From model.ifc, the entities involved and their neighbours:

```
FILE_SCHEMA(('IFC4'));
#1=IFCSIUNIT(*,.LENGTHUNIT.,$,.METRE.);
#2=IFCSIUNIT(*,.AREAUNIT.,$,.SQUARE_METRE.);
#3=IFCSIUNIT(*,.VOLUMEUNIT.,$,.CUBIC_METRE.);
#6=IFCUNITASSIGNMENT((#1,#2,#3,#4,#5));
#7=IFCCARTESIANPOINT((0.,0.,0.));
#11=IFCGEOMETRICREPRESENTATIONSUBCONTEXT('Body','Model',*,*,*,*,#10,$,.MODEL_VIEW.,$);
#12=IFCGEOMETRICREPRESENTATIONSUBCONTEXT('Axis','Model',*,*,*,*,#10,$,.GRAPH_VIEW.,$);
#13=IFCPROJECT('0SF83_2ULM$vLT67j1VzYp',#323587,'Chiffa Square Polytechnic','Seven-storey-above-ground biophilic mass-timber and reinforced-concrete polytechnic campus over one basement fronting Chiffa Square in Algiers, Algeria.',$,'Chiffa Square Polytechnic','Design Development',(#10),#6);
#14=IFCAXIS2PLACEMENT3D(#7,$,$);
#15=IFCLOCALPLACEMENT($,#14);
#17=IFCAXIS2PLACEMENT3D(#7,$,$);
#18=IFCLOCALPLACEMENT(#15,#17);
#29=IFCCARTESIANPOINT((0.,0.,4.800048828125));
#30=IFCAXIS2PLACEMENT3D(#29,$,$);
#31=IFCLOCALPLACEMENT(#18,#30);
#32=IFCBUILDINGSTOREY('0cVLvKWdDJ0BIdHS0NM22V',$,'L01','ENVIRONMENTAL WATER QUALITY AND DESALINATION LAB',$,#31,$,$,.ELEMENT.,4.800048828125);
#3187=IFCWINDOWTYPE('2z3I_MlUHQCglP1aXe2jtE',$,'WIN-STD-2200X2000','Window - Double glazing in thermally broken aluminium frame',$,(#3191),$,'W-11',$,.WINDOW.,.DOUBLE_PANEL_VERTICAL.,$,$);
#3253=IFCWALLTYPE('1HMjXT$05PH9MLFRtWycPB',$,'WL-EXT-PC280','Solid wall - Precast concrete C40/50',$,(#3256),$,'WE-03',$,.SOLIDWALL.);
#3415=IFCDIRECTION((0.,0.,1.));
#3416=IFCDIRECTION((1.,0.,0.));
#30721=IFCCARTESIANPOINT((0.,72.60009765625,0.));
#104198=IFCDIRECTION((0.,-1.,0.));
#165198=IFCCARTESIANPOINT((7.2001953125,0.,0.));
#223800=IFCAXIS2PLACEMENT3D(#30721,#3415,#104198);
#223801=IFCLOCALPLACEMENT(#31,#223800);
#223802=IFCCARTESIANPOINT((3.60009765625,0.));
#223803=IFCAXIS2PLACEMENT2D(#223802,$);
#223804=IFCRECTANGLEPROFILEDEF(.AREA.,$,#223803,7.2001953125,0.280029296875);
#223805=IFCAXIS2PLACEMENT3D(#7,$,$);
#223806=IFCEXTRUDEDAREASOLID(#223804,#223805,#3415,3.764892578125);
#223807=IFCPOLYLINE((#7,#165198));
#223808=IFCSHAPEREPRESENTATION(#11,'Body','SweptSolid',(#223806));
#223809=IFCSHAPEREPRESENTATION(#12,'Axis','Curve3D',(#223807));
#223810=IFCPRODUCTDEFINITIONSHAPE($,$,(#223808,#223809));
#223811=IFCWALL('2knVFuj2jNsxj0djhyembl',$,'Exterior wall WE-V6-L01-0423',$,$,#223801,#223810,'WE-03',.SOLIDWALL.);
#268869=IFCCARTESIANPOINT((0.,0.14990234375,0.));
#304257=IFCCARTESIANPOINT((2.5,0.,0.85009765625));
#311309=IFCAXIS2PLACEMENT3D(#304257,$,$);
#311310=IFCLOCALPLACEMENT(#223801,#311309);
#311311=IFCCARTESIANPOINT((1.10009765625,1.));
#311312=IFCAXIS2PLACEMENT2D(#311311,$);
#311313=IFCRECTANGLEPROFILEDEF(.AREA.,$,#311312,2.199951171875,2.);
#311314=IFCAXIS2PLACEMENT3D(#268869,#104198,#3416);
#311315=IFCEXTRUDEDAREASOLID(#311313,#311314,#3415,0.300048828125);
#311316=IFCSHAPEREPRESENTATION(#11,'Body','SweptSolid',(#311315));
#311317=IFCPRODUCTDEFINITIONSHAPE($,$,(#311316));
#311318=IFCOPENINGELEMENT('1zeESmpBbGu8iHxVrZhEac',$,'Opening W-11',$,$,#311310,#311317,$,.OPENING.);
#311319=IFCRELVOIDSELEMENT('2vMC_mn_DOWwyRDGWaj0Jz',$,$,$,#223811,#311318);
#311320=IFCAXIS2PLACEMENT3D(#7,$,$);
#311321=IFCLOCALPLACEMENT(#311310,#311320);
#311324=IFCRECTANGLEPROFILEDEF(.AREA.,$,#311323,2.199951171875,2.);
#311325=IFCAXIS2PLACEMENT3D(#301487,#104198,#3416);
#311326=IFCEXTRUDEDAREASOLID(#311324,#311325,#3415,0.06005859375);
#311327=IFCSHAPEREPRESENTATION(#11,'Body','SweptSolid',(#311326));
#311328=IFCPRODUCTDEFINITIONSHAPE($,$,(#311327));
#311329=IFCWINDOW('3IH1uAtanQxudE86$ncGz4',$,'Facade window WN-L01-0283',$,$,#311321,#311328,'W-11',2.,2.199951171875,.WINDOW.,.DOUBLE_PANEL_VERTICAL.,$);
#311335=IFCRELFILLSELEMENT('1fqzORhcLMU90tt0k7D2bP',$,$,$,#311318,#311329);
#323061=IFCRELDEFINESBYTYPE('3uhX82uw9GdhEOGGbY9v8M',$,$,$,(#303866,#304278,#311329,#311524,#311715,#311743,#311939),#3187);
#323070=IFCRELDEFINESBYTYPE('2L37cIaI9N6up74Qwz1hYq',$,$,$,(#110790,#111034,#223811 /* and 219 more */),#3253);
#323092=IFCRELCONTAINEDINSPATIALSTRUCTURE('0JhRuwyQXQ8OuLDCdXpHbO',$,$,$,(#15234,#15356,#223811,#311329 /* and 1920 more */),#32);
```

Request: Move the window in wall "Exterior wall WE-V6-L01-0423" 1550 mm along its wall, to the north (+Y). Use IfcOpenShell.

```python
import ifcopenshell
import ifcopenshell.api.geometry
import ifcopenshell.util.placement
import ifcopenshell.util.unit

model = ifcopenshell.open("model.ifc")
unit_scale = ifcopenshell.util.unit.calculate_unit_scale(model)

window = model.by_guid("3IH1uAtanQxudE86$ncGz4")
opening = window.FillsVoids[0].RelatingOpeningElement
wall = opening.VoidsElements[0].RelatingBuildingElement

wall_matrix = ifcopenshell.util.placement.get_local_placement(wall.ObjectPlacement)
shift = wall_matrix[:3, 0] * -1.55 / unit_scale
before = ifcopenshell.util.placement.get_local_placement(window.ObjectPlacement)[:3, 3].copy()

# The window is placed relative to its opening, so it follows when the opening moves.
matrix = ifcopenshell.util.placement.get_local_placement(opening.ObjectPlacement)
matrix[:3, 3] += shift
ifcopenshell.api.geometry.edit_object_placement(
    model, product=opening, matrix=matrix, is_si=False, should_transform_children=True
)

after = ifcopenshell.util.placement.get_local_placement(window.ObjectPlacement)[:3, 3]
print("window moved by", (after - before).round(3) + 0.0)

model.write("model-out.ifc")
```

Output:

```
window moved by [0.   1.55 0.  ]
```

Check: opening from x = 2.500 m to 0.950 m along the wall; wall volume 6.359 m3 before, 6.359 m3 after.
